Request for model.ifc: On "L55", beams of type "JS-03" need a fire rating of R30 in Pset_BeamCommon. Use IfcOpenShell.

First a look at what the model holds.

```python
import ifcopenshell
import ifcopenshell.util.element

model = ifcopenshell.open("model.ifc")
print(model.schema)
storey = next(s for s in model.by_type("IfcBuildingStorey") if s.Name == "L55")
beams = [e for e in ifcopenshell.util.element.get_decomposition(storey) if e.is_a("IfcBeam")]
seen = {}
for e in beams:
    element_type = ifcopenshell.util.element.get_type(e)
    key = (element_type.Name if element_type != e and element_type else None, ifcopenshell.util.element.get_pset(e, "Pset_BeamCommon", "FireRating"))
    seen[key] = seen.get(key, 0) + 1
for (name, value), count in sorted(seen.items(), key=str):
    print(count, "x", name, "|", value)
```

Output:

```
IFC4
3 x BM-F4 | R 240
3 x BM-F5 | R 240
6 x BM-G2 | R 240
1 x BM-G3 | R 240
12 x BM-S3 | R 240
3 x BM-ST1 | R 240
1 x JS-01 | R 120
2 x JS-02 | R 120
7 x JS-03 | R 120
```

```python
import ifcopenshell
import ifcopenshell.api.pset
import ifcopenshell.util.element

model = ifcopenshell.open("model.ifc")

storey = next(s for s in model.by_type("IfcBuildingStorey") if s.Name == "L55")
beams = [e for e in ifcopenshell.util.element.get_decomposition(storey) if e.is_a("IfcBeam")]

count = 0
for e in beams:
    element_type = ifcopenshell.util.element.get_type(e)
    if element_type in (None, e) or element_type.Name != "JS-03":
        continue
    # add_pset returns the element's existing set when there is one.
    pset = ifcopenshell.api.pset.add_pset(model, product=e, name="Pset_BeamCommon")
    ifcopenshell.api.pset.edit_pset(model, pset=pset, properties={"FireRating": "R30"})
    count += 1

print(count, "beams updated")

model.write("model_updated.ifc")
```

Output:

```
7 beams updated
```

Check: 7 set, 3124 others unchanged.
